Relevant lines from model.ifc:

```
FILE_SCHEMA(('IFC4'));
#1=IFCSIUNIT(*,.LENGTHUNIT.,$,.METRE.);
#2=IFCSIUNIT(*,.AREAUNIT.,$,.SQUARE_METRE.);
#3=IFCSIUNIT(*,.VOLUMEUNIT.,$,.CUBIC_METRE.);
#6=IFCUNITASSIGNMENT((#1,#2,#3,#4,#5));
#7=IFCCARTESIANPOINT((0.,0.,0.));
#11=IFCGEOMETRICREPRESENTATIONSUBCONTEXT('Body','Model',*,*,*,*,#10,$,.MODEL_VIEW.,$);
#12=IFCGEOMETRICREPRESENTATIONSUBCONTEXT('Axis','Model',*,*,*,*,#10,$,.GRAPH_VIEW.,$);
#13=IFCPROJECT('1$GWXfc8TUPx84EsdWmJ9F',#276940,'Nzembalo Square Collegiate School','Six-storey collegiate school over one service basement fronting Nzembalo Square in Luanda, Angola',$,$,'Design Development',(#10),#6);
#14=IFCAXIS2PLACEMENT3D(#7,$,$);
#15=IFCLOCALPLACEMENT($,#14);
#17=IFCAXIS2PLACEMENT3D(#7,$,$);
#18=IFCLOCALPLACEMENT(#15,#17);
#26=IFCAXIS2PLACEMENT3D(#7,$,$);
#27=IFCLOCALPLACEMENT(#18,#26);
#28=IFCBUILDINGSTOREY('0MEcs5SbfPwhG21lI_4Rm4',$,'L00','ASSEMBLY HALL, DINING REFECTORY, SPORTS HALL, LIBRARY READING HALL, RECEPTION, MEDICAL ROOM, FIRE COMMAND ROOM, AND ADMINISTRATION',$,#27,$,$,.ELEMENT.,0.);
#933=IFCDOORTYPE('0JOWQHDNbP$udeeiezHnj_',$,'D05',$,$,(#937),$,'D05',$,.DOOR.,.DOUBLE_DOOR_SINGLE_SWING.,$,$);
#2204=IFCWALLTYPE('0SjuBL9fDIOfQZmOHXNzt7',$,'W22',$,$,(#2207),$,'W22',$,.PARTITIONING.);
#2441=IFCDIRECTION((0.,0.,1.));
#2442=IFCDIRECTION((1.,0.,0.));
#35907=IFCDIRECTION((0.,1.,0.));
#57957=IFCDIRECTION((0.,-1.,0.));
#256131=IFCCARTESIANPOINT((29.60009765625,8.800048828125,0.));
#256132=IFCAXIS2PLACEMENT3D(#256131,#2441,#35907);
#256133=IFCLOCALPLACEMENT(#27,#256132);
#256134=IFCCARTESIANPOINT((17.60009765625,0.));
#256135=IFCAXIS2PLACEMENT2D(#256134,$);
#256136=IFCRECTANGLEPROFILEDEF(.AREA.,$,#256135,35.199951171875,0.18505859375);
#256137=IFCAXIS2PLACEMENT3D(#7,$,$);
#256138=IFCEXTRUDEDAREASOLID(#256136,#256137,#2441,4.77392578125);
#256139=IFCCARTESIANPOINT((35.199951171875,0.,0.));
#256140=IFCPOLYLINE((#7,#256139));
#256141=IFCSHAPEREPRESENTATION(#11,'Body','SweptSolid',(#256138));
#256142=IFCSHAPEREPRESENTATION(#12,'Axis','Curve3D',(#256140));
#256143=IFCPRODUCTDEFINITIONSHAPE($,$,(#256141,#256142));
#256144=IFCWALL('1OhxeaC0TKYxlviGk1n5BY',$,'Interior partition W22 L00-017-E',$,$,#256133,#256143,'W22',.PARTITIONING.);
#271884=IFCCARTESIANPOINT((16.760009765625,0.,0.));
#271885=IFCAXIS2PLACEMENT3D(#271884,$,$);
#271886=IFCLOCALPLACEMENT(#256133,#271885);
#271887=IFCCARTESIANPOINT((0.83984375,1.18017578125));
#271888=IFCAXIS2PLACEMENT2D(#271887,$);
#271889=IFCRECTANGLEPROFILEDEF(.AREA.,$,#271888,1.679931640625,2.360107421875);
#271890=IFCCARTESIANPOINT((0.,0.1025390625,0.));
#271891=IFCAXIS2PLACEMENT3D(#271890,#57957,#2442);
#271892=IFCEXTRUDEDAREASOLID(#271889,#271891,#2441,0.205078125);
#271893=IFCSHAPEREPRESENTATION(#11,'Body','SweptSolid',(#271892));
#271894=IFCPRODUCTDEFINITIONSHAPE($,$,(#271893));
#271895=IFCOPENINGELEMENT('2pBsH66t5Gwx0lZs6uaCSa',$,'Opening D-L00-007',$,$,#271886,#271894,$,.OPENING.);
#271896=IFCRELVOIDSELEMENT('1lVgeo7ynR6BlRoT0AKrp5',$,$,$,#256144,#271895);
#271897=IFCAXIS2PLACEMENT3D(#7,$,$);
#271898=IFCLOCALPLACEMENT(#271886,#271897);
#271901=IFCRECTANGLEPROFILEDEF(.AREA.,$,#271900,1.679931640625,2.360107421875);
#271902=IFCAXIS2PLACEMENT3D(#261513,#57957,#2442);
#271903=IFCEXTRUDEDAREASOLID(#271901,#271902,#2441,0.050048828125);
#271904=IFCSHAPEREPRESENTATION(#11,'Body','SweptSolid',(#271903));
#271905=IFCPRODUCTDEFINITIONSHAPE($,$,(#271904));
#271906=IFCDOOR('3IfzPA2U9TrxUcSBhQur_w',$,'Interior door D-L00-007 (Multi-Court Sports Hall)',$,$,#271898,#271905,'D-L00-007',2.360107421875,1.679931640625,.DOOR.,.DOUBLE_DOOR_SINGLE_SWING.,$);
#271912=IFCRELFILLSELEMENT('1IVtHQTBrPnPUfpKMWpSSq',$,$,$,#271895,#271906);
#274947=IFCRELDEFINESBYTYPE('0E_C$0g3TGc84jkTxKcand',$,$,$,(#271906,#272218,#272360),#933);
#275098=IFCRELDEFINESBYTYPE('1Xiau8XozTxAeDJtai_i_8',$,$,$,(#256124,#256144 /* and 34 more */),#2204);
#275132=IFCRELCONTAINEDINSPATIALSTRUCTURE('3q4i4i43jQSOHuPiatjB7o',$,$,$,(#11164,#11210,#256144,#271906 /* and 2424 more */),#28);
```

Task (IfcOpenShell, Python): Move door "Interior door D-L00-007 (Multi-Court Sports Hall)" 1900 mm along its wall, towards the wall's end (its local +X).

```python
import ifcopenshell
import ifcopenshell.api.geometry
import ifcopenshell.util.placement
import ifcopenshell.util.unit

model = ifcopenshell.open("model.ifc")
unit_scale = ifcopenshell.util.unit.calculate_unit_scale(model)

door = model.by_guid("3IfzPA2U9TrxUcSBhQur_w")
opening = door.FillsVoids[0].RelatingOpeningElement
wall = opening.VoidsElements[0].RelatingBuildingElement

wall_matrix = ifcopenshell.util.placement.get_local_placement(wall.ObjectPlacement)
shift = wall_matrix[:3, 0] * 1.9 / unit_scale
before = ifcopenshell.util.placement.get_local_placement(door.ObjectPlacement)[:3, 3].copy()

# The door is placed relative to its opening, so it follows when the opening moves.
matrix = ifcopenshell.util.placement.get_local_placement(opening.ObjectPlacement)
matrix[:3, 3] += shift
ifcopenshell.api.geometry.edit_object_placement(
    model, product=opening, matrix=matrix, is_si=False, should_transform_children=True
)

after = ifcopenshell.util.placement.get_local_placement(door.ObjectPlacement)[:3, 3]
print("door moved by", (after - before).round(3) + 0.0)

model.write("model_edited.ifc")
```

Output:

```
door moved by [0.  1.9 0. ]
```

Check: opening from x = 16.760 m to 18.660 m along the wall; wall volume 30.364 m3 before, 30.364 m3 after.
